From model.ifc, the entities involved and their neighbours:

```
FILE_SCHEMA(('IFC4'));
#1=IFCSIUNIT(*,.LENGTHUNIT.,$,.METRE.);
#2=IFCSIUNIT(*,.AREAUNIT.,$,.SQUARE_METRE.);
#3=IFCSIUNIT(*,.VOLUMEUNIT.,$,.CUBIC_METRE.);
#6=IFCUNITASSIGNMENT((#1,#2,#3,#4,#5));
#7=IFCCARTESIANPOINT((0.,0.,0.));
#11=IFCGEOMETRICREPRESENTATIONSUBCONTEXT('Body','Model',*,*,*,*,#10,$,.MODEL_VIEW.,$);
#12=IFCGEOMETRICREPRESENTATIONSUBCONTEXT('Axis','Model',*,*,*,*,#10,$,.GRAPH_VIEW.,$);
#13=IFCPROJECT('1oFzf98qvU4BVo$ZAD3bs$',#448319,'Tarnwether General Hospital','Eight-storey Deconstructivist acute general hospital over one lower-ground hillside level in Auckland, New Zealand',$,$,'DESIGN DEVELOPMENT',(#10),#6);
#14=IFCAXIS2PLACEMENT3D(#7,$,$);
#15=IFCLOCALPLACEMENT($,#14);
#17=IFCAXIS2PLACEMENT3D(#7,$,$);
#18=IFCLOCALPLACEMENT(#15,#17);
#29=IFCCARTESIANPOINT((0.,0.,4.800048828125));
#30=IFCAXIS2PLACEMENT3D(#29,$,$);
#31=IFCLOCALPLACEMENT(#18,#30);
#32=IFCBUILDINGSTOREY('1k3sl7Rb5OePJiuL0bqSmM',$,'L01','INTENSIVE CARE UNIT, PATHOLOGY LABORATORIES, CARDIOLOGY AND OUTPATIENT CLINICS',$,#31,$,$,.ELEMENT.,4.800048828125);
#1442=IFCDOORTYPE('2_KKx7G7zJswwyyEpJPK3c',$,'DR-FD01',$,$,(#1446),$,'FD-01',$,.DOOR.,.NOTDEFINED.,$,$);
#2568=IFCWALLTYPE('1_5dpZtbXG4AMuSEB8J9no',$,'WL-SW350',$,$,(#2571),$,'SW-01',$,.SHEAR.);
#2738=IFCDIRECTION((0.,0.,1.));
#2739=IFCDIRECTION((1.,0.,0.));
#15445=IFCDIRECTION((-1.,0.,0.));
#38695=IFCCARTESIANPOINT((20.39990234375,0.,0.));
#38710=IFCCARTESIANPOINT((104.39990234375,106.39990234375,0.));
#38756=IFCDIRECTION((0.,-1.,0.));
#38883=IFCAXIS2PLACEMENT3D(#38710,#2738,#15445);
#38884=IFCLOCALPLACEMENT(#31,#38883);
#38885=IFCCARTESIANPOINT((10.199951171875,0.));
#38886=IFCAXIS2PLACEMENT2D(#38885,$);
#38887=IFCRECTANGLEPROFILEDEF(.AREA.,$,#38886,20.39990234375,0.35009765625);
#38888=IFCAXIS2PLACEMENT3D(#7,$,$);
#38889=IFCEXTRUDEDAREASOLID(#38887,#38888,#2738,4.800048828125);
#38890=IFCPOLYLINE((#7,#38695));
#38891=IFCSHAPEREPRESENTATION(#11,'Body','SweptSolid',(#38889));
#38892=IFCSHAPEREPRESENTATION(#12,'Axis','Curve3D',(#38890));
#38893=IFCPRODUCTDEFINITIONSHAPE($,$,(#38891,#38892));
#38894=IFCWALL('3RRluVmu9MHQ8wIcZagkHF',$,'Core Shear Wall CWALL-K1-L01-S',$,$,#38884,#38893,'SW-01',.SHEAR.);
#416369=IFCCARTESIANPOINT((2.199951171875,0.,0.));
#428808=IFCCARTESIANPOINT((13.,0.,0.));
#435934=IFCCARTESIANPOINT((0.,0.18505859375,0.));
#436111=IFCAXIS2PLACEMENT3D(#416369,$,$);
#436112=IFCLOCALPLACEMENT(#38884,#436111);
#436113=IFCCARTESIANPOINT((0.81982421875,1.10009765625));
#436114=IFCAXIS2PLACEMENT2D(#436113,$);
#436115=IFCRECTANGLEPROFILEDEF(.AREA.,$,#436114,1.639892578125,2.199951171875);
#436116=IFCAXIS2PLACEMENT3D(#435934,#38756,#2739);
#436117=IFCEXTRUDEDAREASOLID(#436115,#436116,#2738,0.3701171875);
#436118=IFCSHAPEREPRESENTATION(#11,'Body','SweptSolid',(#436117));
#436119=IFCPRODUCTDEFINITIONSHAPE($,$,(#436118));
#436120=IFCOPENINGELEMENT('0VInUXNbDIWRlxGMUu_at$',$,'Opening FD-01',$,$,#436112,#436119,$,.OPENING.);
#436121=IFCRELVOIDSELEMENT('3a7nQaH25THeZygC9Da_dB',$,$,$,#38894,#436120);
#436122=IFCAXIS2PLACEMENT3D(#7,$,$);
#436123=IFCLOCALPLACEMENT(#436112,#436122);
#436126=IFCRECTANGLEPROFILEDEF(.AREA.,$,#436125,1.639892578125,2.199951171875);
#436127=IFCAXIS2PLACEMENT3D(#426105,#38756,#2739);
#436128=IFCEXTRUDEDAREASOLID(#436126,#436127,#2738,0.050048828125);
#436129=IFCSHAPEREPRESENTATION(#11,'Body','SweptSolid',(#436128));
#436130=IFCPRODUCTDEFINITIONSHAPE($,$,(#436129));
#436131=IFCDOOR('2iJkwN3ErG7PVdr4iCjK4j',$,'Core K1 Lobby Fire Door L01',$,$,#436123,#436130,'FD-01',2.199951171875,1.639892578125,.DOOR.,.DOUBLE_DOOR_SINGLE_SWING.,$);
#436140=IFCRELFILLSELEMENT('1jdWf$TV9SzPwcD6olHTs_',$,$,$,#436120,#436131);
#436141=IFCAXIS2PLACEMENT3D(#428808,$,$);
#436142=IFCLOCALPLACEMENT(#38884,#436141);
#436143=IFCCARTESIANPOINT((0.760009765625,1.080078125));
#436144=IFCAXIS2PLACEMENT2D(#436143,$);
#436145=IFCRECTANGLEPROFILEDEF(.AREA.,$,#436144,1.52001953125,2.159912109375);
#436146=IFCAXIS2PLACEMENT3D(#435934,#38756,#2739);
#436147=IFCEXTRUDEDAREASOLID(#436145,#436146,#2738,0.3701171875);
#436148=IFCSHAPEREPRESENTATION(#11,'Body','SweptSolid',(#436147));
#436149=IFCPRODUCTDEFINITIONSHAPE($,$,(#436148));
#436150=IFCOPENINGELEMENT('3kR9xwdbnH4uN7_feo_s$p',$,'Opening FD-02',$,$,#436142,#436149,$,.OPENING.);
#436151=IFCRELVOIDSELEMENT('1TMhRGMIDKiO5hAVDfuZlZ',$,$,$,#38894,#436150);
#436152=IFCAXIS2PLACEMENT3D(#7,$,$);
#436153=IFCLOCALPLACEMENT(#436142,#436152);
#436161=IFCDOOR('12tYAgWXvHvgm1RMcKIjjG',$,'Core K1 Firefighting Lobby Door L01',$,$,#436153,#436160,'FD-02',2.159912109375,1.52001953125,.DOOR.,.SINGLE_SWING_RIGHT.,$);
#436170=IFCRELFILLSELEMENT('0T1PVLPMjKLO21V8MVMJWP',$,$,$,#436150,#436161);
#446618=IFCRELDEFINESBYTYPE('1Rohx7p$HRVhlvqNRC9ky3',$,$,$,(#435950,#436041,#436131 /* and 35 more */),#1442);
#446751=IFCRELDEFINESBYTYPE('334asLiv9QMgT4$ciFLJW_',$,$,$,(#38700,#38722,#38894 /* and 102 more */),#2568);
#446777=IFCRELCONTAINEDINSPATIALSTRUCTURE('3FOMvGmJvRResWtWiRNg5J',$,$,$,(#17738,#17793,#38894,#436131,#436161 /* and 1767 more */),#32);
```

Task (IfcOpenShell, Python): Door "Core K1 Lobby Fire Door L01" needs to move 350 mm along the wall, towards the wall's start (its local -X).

```python
import ifcopenshell
import ifcopenshell.api.geometry
import ifcopenshell.util.placement
import ifcopenshell.util.unit

model = ifcopenshell.open("model.ifc")
unit_scale = ifcopenshell.util.unit.calculate_unit_scale(model)

door = model.by_guid("2iJkwN3ErG7PVdr4iCjK4j")
opening = door.FillsVoids[0].RelatingOpeningElement
wall = opening.VoidsElements[0].RelatingBuildingElement

wall_matrix = ifcopenshell.util.placement.get_local_placement(wall.ObjectPlacement)
shift = wall_matrix[:3, 0] * -0.35 / unit_scale
before = ifcopenshell.util.placement.get_local_placement(door.ObjectPlacement)[:3, 3].copy()

# The door is placed relative to its opening, so it follows when the opening moves.
matrix = ifcopenshell.util.placement.get_local_placement(opening.ObjectPlacement)
matrix[:3, 3] += shift
ifcopenshell.api.geometry.edit_object_placement(
    model, product=opening, matrix=matrix, is_si=False, should_transform_children=True
)

after = ifcopenshell.util.placement.get_local_placement(door.ObjectPlacement)[:3, 3]
print("door moved by", (after - before).round(3) + 0.0)

model.write("model-out.ifc")
```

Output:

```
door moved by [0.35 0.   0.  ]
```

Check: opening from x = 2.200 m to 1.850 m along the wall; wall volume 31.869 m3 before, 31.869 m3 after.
